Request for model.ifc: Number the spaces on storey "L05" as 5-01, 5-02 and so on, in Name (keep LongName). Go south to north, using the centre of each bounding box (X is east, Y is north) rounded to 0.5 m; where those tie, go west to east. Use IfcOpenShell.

First a look at what the model holds.

```python
import ifcopenshell
import ifcopenshell.util.element
import ifcopenshell.util.placement

model = ifcopenshell.open("model.ifc")
print(model.schema)
storey = next(s for s in model.by_type("IfcBuildingStorey") if s.Name == "L05")
spaces = [e for e in ifcopenshell.util.element.get_decomposition(storey) if e.is_a("IfcSpace")]
for e in sorted(spaces, key=lambda e: e.id()):
    origin = ifcopenshell.util.placement.get_local_placement(e.ObjectPlacement)[:3, 3]
    print(e.id(), e.Name, e.LongName, origin.round(2) + 0.0, sep=" | ")
```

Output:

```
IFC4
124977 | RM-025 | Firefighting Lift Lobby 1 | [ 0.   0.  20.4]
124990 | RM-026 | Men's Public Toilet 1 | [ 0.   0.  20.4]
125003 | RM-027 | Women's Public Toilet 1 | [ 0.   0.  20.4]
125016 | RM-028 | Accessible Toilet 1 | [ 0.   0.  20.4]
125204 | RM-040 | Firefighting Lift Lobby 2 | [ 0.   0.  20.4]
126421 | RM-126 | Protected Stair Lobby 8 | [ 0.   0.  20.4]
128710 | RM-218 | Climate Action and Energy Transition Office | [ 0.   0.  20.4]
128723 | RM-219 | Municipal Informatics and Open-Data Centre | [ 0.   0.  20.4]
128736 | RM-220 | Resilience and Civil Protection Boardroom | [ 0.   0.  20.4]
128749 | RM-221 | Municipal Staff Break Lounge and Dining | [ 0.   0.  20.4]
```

```python
import ifcopenshell
import ifcopenshell.geom
import ifcopenshell.util.element
import ifcopenshell.util.shape

model = ifcopenshell.open("model.ifc")
settings = ifcopenshell.geom.settings()
settings.set("use-world-coords", True)


def centre(element):
    shape = ifcopenshell.geom.create_shape(settings, element)
    return ifcopenshell.util.shape.get_bbox_centroid(shape.geometry)


storey = next(s for s in model.by_type("IfcBuildingStorey") if s.Name == "L05")
spaces = [e for e in ifcopenshell.util.element.get_decomposition(storey) if e.is_a("IfcSpace")]

# Insertion points can sit at a corner or the storey origin, so sort by the geometry (in metres).
centres = {e: centre(e) for e in spaces}
spaces.sort(key=lambda e: (round(centres[e][1] / 0.5), centres[e][0]))

for i, e in enumerate(spaces, start=1):
    number = f"5-{i:02d}"
    e.Name = number
    print(e.id(), number)

model.write("model_edited.ifc")
```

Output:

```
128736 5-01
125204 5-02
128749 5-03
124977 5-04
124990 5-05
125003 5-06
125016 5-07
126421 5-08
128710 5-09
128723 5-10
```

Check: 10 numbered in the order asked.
